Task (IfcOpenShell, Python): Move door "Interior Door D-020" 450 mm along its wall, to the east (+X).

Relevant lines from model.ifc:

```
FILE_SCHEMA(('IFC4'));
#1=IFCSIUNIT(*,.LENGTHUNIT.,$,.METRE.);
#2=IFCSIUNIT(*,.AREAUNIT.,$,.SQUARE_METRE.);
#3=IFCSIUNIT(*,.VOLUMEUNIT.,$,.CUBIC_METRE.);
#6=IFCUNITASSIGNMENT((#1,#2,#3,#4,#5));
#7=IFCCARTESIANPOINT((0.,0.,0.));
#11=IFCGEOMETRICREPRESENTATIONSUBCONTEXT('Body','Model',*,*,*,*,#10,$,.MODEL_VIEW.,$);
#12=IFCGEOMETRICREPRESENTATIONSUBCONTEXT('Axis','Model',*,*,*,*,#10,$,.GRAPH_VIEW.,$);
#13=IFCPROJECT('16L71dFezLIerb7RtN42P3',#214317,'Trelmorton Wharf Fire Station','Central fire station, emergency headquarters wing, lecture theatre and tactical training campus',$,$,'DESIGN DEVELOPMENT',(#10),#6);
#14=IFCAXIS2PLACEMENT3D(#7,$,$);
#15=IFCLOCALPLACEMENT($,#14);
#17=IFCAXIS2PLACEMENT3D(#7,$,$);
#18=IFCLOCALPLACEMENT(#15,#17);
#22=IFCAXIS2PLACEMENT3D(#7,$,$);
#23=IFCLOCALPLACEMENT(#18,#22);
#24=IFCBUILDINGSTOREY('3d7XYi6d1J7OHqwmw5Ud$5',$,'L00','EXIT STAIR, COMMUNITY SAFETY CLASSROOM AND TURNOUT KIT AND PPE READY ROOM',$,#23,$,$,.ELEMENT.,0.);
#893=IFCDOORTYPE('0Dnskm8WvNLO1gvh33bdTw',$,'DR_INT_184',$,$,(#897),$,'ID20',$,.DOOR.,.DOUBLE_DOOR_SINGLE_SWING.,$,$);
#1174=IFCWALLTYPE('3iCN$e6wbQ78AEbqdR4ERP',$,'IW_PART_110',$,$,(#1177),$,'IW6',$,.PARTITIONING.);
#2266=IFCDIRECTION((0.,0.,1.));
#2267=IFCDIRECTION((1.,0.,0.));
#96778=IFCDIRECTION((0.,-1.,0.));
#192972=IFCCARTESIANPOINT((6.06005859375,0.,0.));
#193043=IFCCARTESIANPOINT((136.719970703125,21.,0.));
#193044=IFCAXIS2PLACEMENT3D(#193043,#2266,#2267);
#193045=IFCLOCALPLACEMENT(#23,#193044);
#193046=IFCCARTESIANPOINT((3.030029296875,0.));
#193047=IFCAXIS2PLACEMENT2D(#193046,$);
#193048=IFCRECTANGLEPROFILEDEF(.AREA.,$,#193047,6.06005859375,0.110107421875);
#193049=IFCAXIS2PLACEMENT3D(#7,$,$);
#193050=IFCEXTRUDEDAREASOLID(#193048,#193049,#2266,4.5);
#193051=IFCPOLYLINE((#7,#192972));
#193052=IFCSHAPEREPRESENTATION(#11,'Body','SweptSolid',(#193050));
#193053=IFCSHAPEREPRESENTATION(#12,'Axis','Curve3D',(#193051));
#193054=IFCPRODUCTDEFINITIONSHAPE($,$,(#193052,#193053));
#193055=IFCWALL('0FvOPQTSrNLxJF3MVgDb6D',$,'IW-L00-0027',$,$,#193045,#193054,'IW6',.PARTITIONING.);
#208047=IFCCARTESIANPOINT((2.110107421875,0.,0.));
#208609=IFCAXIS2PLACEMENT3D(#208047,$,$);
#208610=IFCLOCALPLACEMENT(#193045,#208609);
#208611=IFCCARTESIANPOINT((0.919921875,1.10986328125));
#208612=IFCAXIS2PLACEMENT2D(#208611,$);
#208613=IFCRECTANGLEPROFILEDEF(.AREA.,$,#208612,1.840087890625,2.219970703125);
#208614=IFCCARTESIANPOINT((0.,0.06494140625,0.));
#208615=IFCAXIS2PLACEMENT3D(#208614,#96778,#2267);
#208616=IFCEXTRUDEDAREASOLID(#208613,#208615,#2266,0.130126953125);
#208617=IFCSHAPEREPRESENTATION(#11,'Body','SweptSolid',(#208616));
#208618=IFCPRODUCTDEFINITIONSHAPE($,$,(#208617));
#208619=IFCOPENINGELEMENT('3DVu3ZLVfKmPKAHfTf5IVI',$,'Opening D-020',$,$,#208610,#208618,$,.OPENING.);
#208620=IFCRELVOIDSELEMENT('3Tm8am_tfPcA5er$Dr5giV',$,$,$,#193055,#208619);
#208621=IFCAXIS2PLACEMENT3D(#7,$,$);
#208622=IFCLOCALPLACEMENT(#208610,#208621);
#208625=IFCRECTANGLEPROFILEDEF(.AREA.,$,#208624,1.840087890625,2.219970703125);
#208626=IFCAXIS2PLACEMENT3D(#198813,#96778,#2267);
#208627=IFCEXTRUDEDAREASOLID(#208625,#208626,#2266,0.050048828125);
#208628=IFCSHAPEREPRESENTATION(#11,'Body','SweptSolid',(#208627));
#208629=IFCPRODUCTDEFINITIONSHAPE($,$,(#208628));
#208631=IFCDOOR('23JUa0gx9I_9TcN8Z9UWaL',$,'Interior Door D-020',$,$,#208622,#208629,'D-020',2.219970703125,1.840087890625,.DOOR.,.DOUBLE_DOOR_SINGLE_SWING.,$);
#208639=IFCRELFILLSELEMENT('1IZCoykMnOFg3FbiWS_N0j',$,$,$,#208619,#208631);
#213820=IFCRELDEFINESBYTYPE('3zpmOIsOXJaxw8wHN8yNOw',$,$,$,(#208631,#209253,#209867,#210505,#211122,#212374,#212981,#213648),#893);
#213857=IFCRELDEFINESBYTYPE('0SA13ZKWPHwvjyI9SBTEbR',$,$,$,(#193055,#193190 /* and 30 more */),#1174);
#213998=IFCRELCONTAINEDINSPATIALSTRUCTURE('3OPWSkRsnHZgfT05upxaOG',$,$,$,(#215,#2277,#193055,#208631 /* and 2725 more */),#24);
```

```python
import ifcopenshell
import ifcopenshell.api.geometry
import ifcopenshell.util.placement

model = ifcopenshell.open("model.ifc")

door = model.by_guid("23JUa0gx9I_9TcN8Z9UWaL")
opening = door.FillsVoids[0].RelatingOpeningElement
wall = opening.VoidsElements[0].RelatingBuildingElement

wall_matrix = ifcopenshell.util.placement.get_local_placement(wall.ObjectPlacement)
shift = wall_matrix[:3, 0] * 0.45
before = ifcopenshell.util.placement.get_local_placement(door.ObjectPlacement)[:3, 3].copy()

# The door is placed relative to its opening, so it follows when the opening moves.
matrix = ifcopenshell.util.placement.get_local_placement(opening.ObjectPlacement)
matrix[:3, 3] += shift
ifcopenshell.api.geometry.edit_object_placement(
    model, product=opening, matrix=matrix, is_si=False, should_transform_children=True
)

after = ifcopenshell.util.placement.get_local_placement(door.ObjectPlacement)[:3, 3]
print("door moved by", (after - before).round(3) + 0.0)

model.write("model_updated.ifc")
```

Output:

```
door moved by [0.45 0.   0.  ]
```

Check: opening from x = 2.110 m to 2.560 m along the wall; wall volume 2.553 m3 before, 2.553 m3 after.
